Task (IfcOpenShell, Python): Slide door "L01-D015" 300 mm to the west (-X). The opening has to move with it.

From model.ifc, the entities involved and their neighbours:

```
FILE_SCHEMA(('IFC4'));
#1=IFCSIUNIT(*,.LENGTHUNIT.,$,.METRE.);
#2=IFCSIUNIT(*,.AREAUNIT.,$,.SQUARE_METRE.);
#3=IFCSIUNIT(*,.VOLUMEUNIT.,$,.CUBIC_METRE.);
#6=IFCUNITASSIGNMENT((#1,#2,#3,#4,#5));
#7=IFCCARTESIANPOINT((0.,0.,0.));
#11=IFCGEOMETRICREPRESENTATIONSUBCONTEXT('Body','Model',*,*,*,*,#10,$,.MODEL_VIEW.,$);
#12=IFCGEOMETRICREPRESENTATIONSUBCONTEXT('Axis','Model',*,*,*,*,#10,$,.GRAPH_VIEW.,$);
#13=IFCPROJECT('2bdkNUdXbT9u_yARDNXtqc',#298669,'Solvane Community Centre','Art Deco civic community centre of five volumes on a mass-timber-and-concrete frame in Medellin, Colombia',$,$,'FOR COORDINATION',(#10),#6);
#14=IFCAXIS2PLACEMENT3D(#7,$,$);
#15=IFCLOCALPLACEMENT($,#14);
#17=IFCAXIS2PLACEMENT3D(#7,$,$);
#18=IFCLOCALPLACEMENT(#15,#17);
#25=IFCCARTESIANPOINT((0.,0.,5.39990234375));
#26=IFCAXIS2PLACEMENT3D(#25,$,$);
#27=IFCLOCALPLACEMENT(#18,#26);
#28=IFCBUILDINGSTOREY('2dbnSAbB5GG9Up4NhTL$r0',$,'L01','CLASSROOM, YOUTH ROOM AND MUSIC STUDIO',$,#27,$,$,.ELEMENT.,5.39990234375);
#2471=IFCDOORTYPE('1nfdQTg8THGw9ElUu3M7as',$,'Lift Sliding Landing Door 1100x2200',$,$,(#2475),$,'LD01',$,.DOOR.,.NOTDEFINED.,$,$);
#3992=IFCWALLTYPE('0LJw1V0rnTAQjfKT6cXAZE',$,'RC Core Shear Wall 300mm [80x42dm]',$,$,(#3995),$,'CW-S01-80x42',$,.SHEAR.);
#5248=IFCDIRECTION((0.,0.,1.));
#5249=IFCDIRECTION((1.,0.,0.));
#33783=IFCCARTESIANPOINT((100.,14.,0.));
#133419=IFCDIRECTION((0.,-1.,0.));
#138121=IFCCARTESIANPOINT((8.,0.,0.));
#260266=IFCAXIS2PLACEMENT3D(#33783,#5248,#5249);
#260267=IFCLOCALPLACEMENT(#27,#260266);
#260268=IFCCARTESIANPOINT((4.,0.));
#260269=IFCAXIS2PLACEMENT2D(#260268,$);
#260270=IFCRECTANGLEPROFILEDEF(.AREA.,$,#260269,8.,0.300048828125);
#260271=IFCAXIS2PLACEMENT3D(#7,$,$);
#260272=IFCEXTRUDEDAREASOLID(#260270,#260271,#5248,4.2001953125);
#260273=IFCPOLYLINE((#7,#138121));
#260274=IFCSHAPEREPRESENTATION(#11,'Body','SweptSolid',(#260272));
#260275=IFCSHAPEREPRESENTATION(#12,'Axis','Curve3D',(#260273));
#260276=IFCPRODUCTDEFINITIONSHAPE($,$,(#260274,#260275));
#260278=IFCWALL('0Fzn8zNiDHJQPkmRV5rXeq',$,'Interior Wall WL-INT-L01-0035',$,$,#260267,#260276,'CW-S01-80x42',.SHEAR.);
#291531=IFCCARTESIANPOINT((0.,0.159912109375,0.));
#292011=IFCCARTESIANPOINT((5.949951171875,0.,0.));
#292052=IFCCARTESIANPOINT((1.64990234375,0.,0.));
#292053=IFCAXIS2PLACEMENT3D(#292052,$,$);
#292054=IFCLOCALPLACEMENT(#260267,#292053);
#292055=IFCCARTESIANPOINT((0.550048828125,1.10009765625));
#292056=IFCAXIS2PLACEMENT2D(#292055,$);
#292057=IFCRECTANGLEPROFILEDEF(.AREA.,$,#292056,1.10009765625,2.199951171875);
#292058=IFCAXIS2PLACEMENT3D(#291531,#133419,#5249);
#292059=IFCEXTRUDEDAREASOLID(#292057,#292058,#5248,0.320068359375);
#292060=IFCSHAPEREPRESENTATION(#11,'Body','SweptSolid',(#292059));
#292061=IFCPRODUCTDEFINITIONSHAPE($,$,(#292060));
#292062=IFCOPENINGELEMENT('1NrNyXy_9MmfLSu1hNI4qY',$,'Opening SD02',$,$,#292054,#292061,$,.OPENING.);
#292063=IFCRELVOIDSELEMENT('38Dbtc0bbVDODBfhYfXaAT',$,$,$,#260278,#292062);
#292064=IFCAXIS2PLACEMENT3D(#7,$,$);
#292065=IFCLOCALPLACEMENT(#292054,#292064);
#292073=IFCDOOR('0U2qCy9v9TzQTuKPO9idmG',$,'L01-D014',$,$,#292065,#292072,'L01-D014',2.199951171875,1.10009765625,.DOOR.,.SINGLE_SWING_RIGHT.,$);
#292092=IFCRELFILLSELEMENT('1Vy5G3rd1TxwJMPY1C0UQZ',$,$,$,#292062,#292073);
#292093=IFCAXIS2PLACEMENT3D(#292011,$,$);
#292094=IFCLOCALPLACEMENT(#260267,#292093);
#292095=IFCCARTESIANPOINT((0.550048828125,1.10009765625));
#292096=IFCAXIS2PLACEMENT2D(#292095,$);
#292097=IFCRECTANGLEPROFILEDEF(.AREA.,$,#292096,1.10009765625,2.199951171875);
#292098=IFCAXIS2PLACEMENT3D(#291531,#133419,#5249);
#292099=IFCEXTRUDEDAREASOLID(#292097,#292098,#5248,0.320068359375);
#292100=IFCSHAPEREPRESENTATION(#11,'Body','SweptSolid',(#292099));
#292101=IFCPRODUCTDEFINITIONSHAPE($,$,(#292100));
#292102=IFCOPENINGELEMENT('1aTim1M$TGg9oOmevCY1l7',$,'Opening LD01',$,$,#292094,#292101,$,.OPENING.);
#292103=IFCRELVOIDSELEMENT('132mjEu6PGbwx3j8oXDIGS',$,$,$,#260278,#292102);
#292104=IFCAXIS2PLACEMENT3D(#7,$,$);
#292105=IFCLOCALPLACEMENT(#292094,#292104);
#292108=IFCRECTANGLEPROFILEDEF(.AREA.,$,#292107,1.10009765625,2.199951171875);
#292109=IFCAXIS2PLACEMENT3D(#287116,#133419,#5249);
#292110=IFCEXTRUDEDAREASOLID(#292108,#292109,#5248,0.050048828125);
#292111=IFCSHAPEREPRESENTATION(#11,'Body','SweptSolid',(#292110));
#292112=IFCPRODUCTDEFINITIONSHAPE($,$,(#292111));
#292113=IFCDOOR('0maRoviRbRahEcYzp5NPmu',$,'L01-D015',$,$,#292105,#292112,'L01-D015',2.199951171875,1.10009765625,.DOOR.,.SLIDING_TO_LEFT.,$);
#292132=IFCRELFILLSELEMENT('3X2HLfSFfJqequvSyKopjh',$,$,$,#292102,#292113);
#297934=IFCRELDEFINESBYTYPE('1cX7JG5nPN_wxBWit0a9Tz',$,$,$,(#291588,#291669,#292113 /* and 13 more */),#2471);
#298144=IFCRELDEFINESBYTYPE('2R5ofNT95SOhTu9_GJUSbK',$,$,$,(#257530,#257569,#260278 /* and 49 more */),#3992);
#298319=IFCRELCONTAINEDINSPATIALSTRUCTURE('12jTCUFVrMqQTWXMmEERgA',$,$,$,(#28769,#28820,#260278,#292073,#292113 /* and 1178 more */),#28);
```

```python
import ifcopenshell
import ifcopenshell.api.geometry
import ifcopenshell.util.placement
import ifcopenshell.util.unit

model = ifcopenshell.open("model.ifc")
unit_scale = ifcopenshell.util.unit.calculate_unit_scale(model)

door = model.by_guid("0maRoviRbRahEcYzp5NPmu")
opening = door.FillsVoids[0].RelatingOpeningElement
wall = opening.VoidsElements[0].RelatingBuildingElement

wall_matrix = ifcopenshell.util.placement.get_local_placement(wall.ObjectPlacement)
shift = wall_matrix[:3, 0] * -0.3 / unit_scale
before = ifcopenshell.util.placement.get_local_placement(door.ObjectPlacement)[:3, 3].copy()

# The door is placed relative to its opening, so it follows when the opening moves.
matrix = ifcopenshell.util.placement.get_local_placement(opening.ObjectPlacement)
matrix[:3, 3] += shift
ifcopenshell.api.geometry.edit_object_placement(
    model, product=opening, matrix=matrix, is_si=False, should_transform_children=True
)

after = ifcopenshell.util.placement.get_local_placement(door.ObjectPlacement)[:3, 3]
print("door moved by", (after - before).round(3) + 0.0)

model.write("model_edited.ifc")
```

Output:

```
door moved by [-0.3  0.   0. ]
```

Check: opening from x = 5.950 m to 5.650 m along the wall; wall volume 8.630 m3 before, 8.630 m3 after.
